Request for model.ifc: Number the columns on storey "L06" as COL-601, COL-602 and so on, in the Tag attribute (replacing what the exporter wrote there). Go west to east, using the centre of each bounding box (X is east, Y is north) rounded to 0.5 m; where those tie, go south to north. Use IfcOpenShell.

First a look at what the model holds.

```python
import ifcopenshell
import ifcopenshell.util.element
import ifcopenshell.util.placement

model = ifcopenshell.open("model.ifc")
print(model.schema)
storey = next(s for s in model.by_type("IfcBuildingStorey") if s.Name == "L06")
columns = [e for e in ifcopenshell.util.element.get_decomposition(storey) if e.is_a("IfcColumn")]
for e in sorted(columns, key=lambda e: e.id()):
    origin = ifcopenshell.util.placement.get_local_placement(e.ObjectPlacement)[:3, 3]
    print(e.id(), e.Tag, e.Name, origin.round(2) + 0.0, sep=" | ")
```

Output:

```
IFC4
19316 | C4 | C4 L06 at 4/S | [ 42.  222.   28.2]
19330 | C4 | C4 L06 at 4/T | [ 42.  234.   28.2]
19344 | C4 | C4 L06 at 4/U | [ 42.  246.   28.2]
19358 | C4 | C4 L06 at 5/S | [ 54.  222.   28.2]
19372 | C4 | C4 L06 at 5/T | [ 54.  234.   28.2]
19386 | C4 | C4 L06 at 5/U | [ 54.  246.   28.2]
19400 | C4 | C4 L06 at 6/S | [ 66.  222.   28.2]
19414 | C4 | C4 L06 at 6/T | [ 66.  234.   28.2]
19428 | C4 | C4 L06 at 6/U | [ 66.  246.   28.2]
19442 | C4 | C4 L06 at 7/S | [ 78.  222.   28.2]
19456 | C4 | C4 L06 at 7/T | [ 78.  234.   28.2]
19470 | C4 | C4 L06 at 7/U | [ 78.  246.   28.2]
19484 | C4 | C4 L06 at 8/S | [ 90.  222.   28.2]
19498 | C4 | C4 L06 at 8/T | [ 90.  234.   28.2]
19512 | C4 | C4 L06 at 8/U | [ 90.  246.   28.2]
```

```python
import ifcopenshell
import ifcopenshell.geom
import ifcopenshell.util.element
import ifcopenshell.util.shape

model = ifcopenshell.open("model.ifc")
settings = ifcopenshell.geom.settings()
settings.set("use-world-coords", True)


def centre(element):
    shape = ifcopenshell.geom.create_shape(settings, element)
    return ifcopenshell.util.shape.get_bbox_centroid(shape.geometry)


storey = next(s for s in model.by_type("IfcBuildingStorey") if s.Name == "L06")
columns = [e for e in ifcopenshell.util.element.get_decomposition(storey) if e.is_a("IfcColumn")]

# Insertion points can sit at a corner or the storey origin, so sort by the geometry (in metres).
centres = {e: centre(e) for e in columns}
columns.sort(key=lambda e: (round(centres[e][0] / 0.5), centres[e][1]))

for i, e in enumerate(columns, start=1):
    number = f"COL-6{i:02d}"
    e.Tag = number
    print(e.id(), number)

model.write("model_edited.ifc")
```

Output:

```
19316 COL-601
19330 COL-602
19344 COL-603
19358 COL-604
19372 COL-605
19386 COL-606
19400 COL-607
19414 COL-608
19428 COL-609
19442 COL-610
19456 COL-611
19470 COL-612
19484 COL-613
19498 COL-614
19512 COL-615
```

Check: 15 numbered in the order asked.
